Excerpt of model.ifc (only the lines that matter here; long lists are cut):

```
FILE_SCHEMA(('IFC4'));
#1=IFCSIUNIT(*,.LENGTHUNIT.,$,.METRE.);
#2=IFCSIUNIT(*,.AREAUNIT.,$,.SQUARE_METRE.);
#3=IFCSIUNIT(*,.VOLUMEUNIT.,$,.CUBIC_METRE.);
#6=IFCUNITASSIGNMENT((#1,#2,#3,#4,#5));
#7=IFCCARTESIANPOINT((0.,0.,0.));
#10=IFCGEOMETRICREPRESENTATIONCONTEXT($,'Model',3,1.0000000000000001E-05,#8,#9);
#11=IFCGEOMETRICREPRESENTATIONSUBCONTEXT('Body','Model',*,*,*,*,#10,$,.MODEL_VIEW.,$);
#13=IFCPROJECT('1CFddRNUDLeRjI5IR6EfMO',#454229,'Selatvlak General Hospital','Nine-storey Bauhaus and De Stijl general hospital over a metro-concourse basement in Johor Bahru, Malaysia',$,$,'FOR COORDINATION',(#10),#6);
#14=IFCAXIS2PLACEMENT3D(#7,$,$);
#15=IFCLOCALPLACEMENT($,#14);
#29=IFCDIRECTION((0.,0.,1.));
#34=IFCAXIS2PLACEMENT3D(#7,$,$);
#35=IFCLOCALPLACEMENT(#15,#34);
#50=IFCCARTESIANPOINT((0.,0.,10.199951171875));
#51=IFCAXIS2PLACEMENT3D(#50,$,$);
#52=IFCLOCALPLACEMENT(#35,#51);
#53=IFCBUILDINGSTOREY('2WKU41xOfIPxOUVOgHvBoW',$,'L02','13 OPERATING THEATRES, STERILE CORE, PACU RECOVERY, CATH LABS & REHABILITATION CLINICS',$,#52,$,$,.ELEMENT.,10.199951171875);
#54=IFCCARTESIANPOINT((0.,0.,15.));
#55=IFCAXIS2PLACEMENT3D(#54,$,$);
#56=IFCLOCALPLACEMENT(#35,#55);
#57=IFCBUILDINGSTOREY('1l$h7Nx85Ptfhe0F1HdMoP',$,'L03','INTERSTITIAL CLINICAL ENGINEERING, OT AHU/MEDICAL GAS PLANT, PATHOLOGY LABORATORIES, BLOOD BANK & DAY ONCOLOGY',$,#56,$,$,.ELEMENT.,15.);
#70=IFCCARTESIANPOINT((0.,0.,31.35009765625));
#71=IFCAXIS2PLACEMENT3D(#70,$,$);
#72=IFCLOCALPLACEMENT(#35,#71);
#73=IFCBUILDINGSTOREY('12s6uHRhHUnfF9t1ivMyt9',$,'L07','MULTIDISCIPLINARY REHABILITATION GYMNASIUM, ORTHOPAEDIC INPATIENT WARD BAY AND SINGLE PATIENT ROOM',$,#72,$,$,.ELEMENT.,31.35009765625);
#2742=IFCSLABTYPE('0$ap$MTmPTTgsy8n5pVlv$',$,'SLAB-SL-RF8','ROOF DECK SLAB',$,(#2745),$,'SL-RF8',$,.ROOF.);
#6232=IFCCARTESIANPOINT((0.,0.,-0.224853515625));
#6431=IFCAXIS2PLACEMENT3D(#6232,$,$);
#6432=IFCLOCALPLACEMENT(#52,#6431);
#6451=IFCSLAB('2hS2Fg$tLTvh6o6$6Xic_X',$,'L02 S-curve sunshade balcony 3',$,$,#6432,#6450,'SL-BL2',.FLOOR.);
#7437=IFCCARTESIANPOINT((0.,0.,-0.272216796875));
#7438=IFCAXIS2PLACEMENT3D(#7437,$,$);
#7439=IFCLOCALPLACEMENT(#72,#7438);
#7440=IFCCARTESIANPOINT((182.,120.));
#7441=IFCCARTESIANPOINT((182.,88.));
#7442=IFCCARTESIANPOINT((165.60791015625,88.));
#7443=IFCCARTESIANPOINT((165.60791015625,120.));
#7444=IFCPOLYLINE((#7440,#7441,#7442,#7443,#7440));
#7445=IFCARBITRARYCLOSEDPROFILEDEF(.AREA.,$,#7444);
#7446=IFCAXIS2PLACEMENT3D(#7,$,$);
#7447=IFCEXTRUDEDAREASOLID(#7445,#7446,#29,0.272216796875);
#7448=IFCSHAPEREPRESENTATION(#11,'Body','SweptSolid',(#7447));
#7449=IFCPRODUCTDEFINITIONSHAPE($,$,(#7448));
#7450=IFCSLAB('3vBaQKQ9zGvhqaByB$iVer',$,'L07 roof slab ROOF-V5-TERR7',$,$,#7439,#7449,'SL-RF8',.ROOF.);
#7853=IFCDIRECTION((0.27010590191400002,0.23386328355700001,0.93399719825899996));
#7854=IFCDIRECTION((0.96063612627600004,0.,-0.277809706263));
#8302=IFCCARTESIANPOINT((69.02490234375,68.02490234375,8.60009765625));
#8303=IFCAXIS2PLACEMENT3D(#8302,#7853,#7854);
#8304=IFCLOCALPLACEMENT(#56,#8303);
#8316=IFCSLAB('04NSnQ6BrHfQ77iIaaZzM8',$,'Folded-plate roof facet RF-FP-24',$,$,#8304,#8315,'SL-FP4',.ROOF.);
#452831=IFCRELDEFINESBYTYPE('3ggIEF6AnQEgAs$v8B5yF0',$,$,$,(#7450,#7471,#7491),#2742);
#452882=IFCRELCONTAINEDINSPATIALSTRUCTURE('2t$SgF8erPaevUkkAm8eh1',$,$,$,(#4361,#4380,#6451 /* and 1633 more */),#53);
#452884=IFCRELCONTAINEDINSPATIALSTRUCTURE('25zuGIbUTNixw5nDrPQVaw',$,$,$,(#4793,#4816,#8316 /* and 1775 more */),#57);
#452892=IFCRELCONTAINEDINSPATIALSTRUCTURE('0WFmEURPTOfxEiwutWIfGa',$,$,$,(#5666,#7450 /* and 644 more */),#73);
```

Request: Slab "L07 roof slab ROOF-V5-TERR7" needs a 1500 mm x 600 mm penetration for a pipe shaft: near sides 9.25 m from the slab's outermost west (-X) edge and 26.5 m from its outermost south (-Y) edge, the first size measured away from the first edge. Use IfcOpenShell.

```python
import numpy as np
import ifcopenshell
import ifcopenshell.api.feature
import ifcopenshell.api.geometry
import ifcopenshell.api.root
import ifcopenshell.geom
import ifcopenshell.util.placement
import ifcopenshell.util.representation
import ifcopenshell.util.shape
import ifcopenshell.util.unit

model = ifcopenshell.open("model.ifc")
unit_scale = ifcopenshell.util.unit.calculate_unit_scale(model)
settings = ifcopenshell.geom.settings()


def volume(element):
    """Net volume in cubic metres, openings subtracted."""
    shape = ifcopenshell.geom.create_shape(settings, element)
    return ifcopenshell.util.shape.get_volume(shape.geometry)


slab = model.by_id(7450)
before = volume(slab)

# Extent in the slab's own axes, in metres. The edges named are its -X and -Y sides.
slab_shape = ifcopenshell.geom.create_shape(settings, slab)
vertices = ifcopenshell.util.shape.get_vertices(slab_shape.geometry)
x_min, y_min, bottom = vertices.min(axis=0)
top = vertices[:, 2].max()

opening = ifcopenshell.api.root.create_entity(model, ifc_class="IfcOpeningElement", name="Pipe shaft opening", predefined_type="OPENING")
context = ifcopenshell.util.representation.get_context(model, "Model", "Body", "MODEL_VIEW")
width, depth = 1.5, 0.6
outline = [(0.0, 0.0), (width, 0.0), (width, depth), (0.0, depth), (0.0, 0.0)]
# Overshoot both faces by 50 mm so the cut is clean.
shape = ifcopenshell.api.geometry.add_slab_representation(
    model, context=context, depth=top - bottom + 0.1, polyline=outline
)
ifcopenshell.api.geometry.assign_representation(model, product=opening, representation=shape)

matrix = ifcopenshell.util.placement.get_local_placement(slab.ObjectPlacement)
matrix[:, 3] = matrix @ np.append(np.array([x_min + 9.25, y_min + 26.5, bottom - 0.05]) / unit_scale, 1.0)
ifcopenshell.api.geometry.edit_object_placement(model, product=opening, matrix=matrix, is_si=False)
ifcopenshell.api.feature.add_feature(model, feature=opening, element=slab)

after = volume(slab)

print(f"slab volume {before:.3f} -> {after:.3f} m3")

model.write("model_edited.ifc")
```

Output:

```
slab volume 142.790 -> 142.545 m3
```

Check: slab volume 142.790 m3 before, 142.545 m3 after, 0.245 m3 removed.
